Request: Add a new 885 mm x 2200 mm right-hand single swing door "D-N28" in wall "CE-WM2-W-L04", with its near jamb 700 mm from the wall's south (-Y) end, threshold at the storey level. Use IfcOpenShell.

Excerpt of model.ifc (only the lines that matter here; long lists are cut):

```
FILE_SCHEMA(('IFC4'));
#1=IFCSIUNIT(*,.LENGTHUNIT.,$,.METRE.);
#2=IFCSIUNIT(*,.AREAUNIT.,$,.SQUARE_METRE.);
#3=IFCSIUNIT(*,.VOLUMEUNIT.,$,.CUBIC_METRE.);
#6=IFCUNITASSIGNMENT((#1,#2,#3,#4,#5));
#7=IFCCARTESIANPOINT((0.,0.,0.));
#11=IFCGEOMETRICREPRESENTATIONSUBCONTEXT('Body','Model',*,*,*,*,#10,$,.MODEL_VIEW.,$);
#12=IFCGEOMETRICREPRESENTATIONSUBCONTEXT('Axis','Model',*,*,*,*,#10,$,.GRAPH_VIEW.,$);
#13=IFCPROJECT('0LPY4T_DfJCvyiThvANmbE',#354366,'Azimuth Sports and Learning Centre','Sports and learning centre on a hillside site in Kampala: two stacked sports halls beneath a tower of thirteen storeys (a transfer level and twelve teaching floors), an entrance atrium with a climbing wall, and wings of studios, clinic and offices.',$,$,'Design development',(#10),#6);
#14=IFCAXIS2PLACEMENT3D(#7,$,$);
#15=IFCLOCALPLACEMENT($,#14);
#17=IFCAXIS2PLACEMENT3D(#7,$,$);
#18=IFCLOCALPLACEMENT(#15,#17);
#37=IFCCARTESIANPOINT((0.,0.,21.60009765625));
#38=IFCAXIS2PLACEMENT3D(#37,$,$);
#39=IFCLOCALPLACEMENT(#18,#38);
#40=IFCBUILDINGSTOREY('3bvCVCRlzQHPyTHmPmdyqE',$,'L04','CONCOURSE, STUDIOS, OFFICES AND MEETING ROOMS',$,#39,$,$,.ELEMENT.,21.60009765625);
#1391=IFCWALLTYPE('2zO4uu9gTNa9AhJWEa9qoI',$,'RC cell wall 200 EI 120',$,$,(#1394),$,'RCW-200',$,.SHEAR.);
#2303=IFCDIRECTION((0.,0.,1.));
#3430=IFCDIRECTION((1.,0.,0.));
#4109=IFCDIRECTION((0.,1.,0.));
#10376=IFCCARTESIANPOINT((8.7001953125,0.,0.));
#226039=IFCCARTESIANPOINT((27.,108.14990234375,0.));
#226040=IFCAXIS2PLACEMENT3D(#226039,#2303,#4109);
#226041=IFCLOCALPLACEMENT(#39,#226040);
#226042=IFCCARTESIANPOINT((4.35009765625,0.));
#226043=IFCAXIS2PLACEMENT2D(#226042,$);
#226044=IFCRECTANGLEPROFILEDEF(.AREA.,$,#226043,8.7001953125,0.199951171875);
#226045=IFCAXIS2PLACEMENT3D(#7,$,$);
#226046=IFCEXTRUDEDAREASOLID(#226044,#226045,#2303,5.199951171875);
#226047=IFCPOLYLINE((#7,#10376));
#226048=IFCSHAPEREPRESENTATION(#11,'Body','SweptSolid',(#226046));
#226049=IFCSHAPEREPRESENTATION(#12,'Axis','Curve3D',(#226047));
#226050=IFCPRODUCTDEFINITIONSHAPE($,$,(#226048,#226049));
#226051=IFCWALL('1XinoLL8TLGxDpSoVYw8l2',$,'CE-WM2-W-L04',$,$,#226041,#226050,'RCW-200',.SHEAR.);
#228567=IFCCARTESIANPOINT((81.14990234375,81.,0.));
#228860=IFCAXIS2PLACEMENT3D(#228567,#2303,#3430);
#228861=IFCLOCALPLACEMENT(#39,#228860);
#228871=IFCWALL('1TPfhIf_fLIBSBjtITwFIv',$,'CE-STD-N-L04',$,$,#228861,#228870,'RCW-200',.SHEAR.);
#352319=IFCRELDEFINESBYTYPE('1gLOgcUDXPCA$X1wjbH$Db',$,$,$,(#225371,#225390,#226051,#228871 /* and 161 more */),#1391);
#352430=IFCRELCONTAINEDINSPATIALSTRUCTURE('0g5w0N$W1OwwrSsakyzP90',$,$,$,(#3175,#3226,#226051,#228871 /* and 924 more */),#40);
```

```python
import numpy as np
import ifcopenshell
import ifcopenshell.api.feature
import ifcopenshell.api.geometry
import ifcopenshell.api.root
import ifcopenshell.api.spatial
import ifcopenshell.geom
import ifcopenshell.util.element
import ifcopenshell.util.placement
import ifcopenshell.util.representation
import ifcopenshell.util.shape
import ifcopenshell.util.unit

model = ifcopenshell.open("model.ifc")
unit_scale = ifcopenshell.util.unit.calculate_unit_scale(model)
settings = ifcopenshell.geom.settings()


def volume(element):
    """Net volume in cubic metres, openings subtracted."""
    shape = ifcopenshell.geom.create_shape(settings, element)
    return ifcopenshell.util.shape.get_volume(shape.geometry)


wall = model.by_id(226051)
storey = ifcopenshell.util.element.get_container(wall, ifc_class="IfcBuildingStorey")
context = ifcopenshell.util.representation.get_context(model, "Model", "Body", "MODEL_VIEW")
before = volume(wall)

width, height, from_end, sill = 0.885, 2.2, 0.7, 0.0  # metres

# The wall runs along its own X axis, and the end named is its -X end.
wall_shape = ifcopenshell.geom.create_shape(settings, wall)
x, y, z = ifcopenshell.util.shape.get_vertices(wall_shape.geometry).T
start = x.min() + from_end
face, thickness = float(y.min()), float(y.max() - y.min())
wall_matrix = ifcopenshell.util.placement.get_local_placement(wall.ObjectPlacement)
level = ifcopenshell.util.placement.get_local_placement(storey.ObjectPlacement)[2, 3]


def in_wall(x, y):
    """Placement at x, y metres in the wall's axes, at sill height."""
    matrix = wall_matrix.copy()
    matrix[:, 3] = wall_matrix @ np.array([x / unit_scale, y / unit_scale, 0.0, 1.0])
    matrix[2, 3] = level + sill / unit_scale
    return matrix


# Opening: a box that overshoots both wall faces by 50 mm.
opening = ifcopenshell.api.root.create_entity(model, ifc_class="IfcOpeningElement", predefined_type="OPENING")
box = ifcopenshell.api.geometry.add_wall_representation(
    model, context=context, length=width, height=height, thickness=thickness + 0.1
)
ifcopenshell.api.geometry.assign_representation(model, product=opening, representation=box)
ifcopenshell.api.geometry.edit_object_placement(model, product=opening, matrix=in_wall(start, face - 0.05), is_si=False)
ifcopenshell.api.feature.add_feature(model, feature=opening, element=wall)

door = ifcopenshell.api.root.create_entity(model, ifc_class="IfcDoor", name="D-N28", predefined_type="DOOR")
door.OverallWidth, door.OverallHeight = width / unit_scale, height / unit_scale
door.OperationType = "SINGLE_SWING_RIGHT"
body = ifcopenshell.api.geometry.add_door_representation(
    model,
    context=context,
    overall_width=door.OverallWidth,
    overall_height=door.OverallHeight,
    operation_type="SINGLE_SWING_RIGHT",
    lining_properties={"LiningDepth": thickness / unit_scale, "ThresholdDepth": thickness / unit_scale},
)
ifcopenshell.api.geometry.assign_representation(model, product=door, representation=body)
ifcopenshell.api.spatial.assign_container(model, products=[door], relating_structure=storey)
ifcopenshell.api.feature.add_filling(model, opening=opening, element=door)

# The lining spans the wall, so the door starts at the wall face.
ifcopenshell.api.geometry.edit_object_placement(model, product=door, matrix=in_wall(start, face), is_si=False)

after = volume(wall)

print(f"wall volume {before:.3f} -> {after:.3f} m3")

model.write("model_updated.ifc")
```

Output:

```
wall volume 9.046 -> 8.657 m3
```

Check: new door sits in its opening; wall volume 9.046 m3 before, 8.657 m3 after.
